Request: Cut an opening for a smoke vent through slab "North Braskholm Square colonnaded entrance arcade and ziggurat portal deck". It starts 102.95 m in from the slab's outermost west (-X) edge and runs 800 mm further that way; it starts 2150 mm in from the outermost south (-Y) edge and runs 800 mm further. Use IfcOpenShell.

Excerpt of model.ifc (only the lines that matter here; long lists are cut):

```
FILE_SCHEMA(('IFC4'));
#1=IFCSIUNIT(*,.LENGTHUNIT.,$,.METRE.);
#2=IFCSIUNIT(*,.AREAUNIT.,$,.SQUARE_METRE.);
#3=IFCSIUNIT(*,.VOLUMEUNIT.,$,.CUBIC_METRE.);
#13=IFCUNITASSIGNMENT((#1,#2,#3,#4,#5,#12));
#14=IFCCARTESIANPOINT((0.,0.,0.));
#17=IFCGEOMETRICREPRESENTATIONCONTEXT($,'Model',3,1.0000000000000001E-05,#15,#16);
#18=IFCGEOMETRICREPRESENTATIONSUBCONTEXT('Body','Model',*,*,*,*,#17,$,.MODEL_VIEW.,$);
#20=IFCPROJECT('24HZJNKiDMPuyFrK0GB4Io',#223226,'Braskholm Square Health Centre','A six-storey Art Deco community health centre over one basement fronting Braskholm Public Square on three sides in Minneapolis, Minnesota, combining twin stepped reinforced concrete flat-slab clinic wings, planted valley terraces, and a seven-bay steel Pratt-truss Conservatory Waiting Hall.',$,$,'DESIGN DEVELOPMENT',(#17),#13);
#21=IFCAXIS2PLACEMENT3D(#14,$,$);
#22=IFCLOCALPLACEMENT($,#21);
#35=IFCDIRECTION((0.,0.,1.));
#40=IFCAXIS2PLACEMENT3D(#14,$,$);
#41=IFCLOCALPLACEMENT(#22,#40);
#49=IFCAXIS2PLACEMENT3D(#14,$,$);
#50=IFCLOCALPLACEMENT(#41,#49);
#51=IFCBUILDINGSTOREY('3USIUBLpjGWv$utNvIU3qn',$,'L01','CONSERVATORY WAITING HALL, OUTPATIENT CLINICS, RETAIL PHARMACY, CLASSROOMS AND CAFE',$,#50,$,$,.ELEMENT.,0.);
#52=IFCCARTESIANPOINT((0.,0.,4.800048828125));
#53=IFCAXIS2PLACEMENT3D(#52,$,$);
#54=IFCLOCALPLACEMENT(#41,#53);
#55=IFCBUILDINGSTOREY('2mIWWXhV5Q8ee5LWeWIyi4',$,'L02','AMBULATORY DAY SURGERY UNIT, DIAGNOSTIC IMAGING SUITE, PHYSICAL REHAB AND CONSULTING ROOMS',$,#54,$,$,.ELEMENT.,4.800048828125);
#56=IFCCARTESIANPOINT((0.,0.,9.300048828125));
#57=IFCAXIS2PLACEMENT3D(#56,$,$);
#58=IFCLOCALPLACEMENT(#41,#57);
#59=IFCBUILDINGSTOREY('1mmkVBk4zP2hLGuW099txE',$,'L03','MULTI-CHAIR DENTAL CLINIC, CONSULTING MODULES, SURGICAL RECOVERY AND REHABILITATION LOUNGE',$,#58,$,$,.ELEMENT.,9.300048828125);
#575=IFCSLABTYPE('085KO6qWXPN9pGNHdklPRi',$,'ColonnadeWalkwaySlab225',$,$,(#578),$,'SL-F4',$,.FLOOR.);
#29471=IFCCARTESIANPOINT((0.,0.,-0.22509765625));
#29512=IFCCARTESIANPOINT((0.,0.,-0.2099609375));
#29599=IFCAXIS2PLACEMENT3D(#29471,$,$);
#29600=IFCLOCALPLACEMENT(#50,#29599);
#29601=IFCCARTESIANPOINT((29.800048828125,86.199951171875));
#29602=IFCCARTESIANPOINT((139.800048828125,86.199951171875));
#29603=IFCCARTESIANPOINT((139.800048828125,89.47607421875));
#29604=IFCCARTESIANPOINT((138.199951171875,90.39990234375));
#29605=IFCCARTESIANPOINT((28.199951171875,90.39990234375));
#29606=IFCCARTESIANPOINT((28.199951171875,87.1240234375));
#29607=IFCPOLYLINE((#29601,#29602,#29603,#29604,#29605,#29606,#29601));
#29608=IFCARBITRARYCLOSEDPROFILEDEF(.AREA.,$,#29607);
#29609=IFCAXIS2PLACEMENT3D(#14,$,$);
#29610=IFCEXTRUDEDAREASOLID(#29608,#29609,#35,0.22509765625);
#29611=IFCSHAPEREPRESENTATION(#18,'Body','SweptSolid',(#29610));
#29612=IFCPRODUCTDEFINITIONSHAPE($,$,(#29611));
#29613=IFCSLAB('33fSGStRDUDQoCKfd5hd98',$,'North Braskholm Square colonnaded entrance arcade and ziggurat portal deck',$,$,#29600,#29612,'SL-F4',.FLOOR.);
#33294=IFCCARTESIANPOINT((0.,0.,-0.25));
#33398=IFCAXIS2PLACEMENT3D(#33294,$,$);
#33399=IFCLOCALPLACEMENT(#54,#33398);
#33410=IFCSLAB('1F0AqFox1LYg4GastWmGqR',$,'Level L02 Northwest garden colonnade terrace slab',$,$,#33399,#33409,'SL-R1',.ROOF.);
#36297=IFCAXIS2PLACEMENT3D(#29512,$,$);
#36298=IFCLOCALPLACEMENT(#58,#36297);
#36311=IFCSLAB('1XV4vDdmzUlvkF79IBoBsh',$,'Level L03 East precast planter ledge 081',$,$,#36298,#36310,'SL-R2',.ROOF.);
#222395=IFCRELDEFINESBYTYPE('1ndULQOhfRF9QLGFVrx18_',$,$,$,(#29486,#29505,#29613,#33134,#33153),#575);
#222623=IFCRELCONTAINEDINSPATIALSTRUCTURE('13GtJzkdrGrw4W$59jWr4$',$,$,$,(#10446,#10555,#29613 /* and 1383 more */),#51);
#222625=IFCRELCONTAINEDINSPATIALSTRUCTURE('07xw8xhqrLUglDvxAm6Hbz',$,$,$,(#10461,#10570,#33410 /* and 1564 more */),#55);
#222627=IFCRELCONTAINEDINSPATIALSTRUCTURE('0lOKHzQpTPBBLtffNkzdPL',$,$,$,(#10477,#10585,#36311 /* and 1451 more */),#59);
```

```python
import numpy as np
import ifcopenshell
import ifcopenshell.api.feature
import ifcopenshell.api.geometry
import ifcopenshell.api.root
import ifcopenshell.geom
import ifcopenshell.util.placement
import ifcopenshell.util.representation
import ifcopenshell.util.shape
import ifcopenshell.util.unit

model = ifcopenshell.open("model.ifc")
unit_scale = ifcopenshell.util.unit.calculate_unit_scale(model)
settings = ifcopenshell.geom.settings()


def volume(element):
    """Net volume in cubic metres, openings subtracted."""
    shape = ifcopenshell.geom.create_shape(settings, element)
    return ifcopenshell.util.shape.get_volume(shape.geometry)


slab = model.by_guid("33fSGStRDUDQoCKfd5hd98")
before = volume(slab)

# Extent in the slab's own axes, in metres. The edges named are its -X and -Y sides.
slab_shape = ifcopenshell.geom.create_shape(settings, slab)
vertices = ifcopenshell.util.shape.get_vertices(slab_shape.geometry)
x_min, y_min, bottom = vertices.min(axis=0)
top = vertices[:, 2].max()

opening = ifcopenshell.api.root.create_entity(model, ifc_class="IfcOpeningElement", name="Smoke vent opening", predefined_type="OPENING")
context = ifcopenshell.util.representation.get_context(model, "Model", "Body", "MODEL_VIEW")
width, depth = 0.8, 0.8
outline = [(0.0, 0.0), (width, 0.0), (width, depth), (0.0, depth), (0.0, 0.0)]
# Overshoot both faces by 50 mm so the cut is clean.
shape = ifcopenshell.api.geometry.add_slab_representation(
    model, context=context, depth=top - bottom + 0.1, polyline=outline
)
ifcopenshell.api.geometry.assign_representation(model, product=opening, representation=shape)

matrix = ifcopenshell.util.placement.get_local_placement(slab.ObjectPlacement)
matrix[:, 3] = matrix @ np.append(np.array([x_min + 102.95, y_min + 2.15, bottom - 0.05]) / unit_scale, 1.0)
ifcopenshell.api.geometry.edit_object_placement(model, product=opening, matrix=matrix, is_si=False)
ifcopenshell.api.feature.add_feature(model, feature=opening, element=slab)

after = volume(slab)

print(f"slab volume {before:.3f} -> {after:.3f} m3")

model.write("model_v2.ifc")
```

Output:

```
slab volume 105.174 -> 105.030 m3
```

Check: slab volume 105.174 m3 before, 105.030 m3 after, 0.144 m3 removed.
